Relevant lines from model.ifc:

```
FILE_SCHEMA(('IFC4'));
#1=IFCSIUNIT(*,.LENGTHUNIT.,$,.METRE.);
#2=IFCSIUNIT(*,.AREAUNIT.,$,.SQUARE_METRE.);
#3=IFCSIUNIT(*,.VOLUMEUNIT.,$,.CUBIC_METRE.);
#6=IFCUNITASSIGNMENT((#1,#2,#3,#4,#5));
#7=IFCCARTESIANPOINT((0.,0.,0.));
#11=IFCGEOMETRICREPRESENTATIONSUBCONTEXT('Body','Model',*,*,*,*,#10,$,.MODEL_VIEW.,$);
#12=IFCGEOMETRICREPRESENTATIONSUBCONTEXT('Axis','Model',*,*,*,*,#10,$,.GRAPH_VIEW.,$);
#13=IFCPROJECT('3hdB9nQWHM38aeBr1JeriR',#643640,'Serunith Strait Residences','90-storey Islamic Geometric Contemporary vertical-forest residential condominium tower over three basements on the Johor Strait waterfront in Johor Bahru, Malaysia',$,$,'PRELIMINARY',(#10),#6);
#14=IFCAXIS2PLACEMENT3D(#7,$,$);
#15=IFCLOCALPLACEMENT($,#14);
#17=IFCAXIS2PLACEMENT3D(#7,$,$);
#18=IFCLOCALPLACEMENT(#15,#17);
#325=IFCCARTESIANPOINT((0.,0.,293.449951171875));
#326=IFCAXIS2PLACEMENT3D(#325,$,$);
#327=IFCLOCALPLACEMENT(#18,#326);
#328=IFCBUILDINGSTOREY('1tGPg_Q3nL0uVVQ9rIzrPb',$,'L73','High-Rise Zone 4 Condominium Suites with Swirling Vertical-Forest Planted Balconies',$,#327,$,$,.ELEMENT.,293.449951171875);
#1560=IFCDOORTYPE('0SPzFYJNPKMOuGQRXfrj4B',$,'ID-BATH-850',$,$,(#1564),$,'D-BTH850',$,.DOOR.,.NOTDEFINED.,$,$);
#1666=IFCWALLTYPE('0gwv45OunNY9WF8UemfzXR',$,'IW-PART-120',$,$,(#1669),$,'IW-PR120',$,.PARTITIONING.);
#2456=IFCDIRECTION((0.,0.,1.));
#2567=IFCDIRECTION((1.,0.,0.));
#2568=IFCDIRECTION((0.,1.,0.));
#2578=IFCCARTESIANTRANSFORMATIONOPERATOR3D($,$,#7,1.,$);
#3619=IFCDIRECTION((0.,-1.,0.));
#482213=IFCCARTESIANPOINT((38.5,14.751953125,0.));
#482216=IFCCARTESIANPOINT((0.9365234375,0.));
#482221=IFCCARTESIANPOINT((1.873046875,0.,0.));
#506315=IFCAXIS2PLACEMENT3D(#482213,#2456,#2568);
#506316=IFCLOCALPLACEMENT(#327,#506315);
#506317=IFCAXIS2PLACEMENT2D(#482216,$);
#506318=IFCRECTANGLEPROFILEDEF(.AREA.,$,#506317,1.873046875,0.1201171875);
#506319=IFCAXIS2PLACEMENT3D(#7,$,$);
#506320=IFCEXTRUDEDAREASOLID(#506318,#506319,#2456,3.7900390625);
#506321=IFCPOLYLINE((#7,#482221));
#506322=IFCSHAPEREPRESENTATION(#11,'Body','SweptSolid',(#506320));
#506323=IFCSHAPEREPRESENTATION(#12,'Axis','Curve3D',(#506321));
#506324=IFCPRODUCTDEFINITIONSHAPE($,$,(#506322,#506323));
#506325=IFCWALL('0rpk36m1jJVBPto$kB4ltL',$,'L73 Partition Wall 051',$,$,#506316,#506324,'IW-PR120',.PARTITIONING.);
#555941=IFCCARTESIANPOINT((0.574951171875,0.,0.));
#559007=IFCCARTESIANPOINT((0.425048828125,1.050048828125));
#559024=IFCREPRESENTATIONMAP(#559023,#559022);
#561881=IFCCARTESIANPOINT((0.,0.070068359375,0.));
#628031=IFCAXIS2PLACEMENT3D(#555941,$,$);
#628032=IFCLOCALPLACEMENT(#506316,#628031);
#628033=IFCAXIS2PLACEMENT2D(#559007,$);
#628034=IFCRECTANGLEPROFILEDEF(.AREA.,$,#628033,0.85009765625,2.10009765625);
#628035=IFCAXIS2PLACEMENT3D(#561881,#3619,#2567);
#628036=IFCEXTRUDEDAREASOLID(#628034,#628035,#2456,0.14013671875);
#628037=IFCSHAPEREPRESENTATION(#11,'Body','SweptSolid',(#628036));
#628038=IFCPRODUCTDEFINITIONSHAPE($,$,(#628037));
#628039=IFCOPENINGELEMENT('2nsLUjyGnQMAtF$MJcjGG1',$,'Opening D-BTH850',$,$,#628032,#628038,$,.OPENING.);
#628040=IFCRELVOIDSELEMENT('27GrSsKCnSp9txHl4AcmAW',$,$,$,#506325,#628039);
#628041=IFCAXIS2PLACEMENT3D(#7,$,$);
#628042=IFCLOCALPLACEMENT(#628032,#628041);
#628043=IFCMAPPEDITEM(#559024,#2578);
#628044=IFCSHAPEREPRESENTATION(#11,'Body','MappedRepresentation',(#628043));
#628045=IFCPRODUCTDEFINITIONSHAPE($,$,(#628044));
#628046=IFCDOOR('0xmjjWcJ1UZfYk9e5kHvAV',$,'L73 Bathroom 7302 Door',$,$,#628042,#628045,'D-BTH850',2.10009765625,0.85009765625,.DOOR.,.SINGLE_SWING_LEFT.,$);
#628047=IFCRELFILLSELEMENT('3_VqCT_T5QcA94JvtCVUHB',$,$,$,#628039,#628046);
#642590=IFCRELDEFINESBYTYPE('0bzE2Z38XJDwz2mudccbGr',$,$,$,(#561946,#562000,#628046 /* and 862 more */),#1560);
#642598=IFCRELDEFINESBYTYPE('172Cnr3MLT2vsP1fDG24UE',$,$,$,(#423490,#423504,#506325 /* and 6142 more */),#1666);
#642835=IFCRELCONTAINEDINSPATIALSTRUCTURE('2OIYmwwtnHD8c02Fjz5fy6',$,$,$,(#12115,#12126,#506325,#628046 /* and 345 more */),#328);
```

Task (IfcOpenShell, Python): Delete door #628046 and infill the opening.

```python
import ifcopenshell
import ifcopenshell.api.feature
import ifcopenshell.api.root
import ifcopenshell.geom
import ifcopenshell.util.shape

model = ifcopenshell.open("model.ifc")
settings = ifcopenshell.geom.settings()


def volume(element):
    """Net volume in cubic metres, openings subtracted."""
    shape = ifcopenshell.geom.create_shape(settings, element)
    return ifcopenshell.util.shape.get_volume(shape.geometry)


door = model.by_id(628046)
opening = door.FillsVoids[0].RelatingOpeningElement
wall = opening.VoidsElements[0].RelatingBuildingElement
before = volume(wall)

ifcopenshell.api.root.remove_product(model, product=door)
ifcopenshell.api.feature.remove_feature(model, feature=opening)

after = volume(wall)

print(f"wall volume {before:.3f} -> {after:.3f} m3")

model.write("model_updated.ifc")
```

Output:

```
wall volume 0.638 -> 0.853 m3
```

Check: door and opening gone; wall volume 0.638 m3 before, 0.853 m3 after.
